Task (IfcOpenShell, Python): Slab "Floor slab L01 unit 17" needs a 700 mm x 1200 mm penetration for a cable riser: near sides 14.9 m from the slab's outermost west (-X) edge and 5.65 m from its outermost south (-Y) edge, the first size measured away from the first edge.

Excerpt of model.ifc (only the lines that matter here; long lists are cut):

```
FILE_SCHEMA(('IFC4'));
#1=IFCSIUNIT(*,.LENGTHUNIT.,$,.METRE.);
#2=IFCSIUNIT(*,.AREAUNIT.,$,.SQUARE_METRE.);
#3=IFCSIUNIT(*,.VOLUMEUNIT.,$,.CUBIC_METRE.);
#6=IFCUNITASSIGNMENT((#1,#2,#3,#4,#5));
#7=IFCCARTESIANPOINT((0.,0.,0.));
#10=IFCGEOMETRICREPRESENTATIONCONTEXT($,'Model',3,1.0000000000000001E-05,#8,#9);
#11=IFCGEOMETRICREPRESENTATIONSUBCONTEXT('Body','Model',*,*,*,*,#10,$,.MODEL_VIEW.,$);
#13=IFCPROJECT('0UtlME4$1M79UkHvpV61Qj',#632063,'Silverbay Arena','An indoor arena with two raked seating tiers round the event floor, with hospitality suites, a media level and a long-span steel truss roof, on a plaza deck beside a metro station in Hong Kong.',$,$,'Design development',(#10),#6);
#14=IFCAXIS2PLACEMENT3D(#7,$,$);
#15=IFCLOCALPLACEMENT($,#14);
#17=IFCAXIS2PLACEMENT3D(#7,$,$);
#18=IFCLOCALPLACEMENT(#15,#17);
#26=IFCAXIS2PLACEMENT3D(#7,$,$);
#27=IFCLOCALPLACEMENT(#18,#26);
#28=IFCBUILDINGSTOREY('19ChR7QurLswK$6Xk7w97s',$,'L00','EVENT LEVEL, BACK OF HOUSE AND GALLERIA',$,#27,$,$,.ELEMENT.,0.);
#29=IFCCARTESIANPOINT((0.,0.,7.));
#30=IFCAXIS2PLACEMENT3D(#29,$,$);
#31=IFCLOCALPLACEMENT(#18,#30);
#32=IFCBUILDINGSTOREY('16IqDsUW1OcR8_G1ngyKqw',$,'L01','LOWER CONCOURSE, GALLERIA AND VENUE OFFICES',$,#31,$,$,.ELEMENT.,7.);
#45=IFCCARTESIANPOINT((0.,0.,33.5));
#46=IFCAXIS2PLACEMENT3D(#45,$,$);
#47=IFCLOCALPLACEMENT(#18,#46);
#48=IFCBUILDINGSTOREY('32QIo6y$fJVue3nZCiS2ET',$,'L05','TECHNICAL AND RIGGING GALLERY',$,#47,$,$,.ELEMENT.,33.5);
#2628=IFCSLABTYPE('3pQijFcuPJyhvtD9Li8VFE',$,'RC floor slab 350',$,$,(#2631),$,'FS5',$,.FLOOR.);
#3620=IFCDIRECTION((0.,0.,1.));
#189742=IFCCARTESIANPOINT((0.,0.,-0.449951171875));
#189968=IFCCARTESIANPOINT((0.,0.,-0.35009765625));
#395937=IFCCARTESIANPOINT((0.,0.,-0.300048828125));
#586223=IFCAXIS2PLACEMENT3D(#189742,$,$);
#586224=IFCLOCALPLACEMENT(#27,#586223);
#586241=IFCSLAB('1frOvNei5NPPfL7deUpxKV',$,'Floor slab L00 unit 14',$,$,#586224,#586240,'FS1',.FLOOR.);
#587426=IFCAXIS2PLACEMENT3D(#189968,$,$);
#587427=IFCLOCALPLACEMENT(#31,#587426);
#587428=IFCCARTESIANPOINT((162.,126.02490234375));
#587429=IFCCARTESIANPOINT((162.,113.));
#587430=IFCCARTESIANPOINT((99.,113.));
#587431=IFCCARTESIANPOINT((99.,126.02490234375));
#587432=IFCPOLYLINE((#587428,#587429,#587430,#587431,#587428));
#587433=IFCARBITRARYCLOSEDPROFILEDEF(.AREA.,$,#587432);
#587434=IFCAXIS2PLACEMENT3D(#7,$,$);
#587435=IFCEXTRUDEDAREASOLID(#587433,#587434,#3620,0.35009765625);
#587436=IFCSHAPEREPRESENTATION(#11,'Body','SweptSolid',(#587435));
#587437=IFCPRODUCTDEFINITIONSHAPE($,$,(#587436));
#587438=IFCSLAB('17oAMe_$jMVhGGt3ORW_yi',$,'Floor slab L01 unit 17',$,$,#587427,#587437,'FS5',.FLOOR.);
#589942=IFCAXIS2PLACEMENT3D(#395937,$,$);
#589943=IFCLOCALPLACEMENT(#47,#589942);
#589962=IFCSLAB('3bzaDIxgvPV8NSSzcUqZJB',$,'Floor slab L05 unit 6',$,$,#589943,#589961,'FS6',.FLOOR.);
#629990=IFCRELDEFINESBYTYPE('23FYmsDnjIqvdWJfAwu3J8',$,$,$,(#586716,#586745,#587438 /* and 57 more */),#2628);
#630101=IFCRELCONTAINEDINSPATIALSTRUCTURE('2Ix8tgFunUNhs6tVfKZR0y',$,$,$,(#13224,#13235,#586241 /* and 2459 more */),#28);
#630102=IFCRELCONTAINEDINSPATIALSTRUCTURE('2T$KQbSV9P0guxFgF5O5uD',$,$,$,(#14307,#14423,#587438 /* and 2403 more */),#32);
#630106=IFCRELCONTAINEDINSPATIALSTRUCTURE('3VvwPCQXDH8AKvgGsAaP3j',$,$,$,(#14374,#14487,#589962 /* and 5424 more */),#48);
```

```python
import numpy as np
import ifcopenshell
import ifcopenshell.api.feature
import ifcopenshell.api.geometry
import ifcopenshell.api.root
import ifcopenshell.geom
import ifcopenshell.util.placement
import ifcopenshell.util.representation
import ifcopenshell.util.shape
import ifcopenshell.util.unit

model = ifcopenshell.open("model.ifc")
unit_scale = ifcopenshell.util.unit.calculate_unit_scale(model)
settings = ifcopenshell.geom.settings()


def volume(element):
    """Net volume in cubic metres, openings subtracted."""
    shape = ifcopenshell.geom.create_shape(settings, element)
    return ifcopenshell.util.shape.get_volume(shape.geometry)


slab = model.by_guid("17oAMe_$jMVhGGt3ORW_yi")
before = volume(slab)

# Extent in the slab's own axes, in metres. The edges named are its -X and -Y sides.
slab_shape = ifcopenshell.geom.create_shape(settings, slab)
vertices = ifcopenshell.util.shape.get_vertices(slab_shape.geometry)
x_min, y_min, bottom = vertices.min(axis=0)
top = vertices[:, 2].max()

opening = ifcopenshell.api.root.create_entity(model, ifc_class="IfcOpeningElement", name="Cable riser opening", predefined_type="OPENING")
context = ifcopenshell.util.representation.get_context(model, "Model", "Body", "MODEL_VIEW")
width, depth = 0.7, 1.2
outline = [(0.0, 0.0), (width, 0.0), (width, depth), (0.0, depth), (0.0, 0.0)]
# Overshoot both faces by 50 mm so the cut is clean.
shape = ifcopenshell.api.geometry.add_slab_representation(
    model, context=context, depth=top - bottom + 0.1, polyline=outline
)
ifcopenshell.api.geometry.assign_representation(model, product=opening, representation=shape)

matrix = ifcopenshell.util.placement.get_local_placement(slab.ObjectPlacement)
matrix[:, 3] = matrix @ np.append(np.array([x_min + 14.9, y_min + 5.65, bottom - 0.05]) / unit_scale, 1.0)
ifcopenshell.api.geometry.edit_object_placement(model, product=opening, matrix=matrix, is_si=False)
ifcopenshell.api.feature.add_feature(model, feature=opening, element=slab)

after = volume(slab)

print(f"slab volume {before:.3f} -> {after:.3f} m3")

model.write("model_edited.ifc")
```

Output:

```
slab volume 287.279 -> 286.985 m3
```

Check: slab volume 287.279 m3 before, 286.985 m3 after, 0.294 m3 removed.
